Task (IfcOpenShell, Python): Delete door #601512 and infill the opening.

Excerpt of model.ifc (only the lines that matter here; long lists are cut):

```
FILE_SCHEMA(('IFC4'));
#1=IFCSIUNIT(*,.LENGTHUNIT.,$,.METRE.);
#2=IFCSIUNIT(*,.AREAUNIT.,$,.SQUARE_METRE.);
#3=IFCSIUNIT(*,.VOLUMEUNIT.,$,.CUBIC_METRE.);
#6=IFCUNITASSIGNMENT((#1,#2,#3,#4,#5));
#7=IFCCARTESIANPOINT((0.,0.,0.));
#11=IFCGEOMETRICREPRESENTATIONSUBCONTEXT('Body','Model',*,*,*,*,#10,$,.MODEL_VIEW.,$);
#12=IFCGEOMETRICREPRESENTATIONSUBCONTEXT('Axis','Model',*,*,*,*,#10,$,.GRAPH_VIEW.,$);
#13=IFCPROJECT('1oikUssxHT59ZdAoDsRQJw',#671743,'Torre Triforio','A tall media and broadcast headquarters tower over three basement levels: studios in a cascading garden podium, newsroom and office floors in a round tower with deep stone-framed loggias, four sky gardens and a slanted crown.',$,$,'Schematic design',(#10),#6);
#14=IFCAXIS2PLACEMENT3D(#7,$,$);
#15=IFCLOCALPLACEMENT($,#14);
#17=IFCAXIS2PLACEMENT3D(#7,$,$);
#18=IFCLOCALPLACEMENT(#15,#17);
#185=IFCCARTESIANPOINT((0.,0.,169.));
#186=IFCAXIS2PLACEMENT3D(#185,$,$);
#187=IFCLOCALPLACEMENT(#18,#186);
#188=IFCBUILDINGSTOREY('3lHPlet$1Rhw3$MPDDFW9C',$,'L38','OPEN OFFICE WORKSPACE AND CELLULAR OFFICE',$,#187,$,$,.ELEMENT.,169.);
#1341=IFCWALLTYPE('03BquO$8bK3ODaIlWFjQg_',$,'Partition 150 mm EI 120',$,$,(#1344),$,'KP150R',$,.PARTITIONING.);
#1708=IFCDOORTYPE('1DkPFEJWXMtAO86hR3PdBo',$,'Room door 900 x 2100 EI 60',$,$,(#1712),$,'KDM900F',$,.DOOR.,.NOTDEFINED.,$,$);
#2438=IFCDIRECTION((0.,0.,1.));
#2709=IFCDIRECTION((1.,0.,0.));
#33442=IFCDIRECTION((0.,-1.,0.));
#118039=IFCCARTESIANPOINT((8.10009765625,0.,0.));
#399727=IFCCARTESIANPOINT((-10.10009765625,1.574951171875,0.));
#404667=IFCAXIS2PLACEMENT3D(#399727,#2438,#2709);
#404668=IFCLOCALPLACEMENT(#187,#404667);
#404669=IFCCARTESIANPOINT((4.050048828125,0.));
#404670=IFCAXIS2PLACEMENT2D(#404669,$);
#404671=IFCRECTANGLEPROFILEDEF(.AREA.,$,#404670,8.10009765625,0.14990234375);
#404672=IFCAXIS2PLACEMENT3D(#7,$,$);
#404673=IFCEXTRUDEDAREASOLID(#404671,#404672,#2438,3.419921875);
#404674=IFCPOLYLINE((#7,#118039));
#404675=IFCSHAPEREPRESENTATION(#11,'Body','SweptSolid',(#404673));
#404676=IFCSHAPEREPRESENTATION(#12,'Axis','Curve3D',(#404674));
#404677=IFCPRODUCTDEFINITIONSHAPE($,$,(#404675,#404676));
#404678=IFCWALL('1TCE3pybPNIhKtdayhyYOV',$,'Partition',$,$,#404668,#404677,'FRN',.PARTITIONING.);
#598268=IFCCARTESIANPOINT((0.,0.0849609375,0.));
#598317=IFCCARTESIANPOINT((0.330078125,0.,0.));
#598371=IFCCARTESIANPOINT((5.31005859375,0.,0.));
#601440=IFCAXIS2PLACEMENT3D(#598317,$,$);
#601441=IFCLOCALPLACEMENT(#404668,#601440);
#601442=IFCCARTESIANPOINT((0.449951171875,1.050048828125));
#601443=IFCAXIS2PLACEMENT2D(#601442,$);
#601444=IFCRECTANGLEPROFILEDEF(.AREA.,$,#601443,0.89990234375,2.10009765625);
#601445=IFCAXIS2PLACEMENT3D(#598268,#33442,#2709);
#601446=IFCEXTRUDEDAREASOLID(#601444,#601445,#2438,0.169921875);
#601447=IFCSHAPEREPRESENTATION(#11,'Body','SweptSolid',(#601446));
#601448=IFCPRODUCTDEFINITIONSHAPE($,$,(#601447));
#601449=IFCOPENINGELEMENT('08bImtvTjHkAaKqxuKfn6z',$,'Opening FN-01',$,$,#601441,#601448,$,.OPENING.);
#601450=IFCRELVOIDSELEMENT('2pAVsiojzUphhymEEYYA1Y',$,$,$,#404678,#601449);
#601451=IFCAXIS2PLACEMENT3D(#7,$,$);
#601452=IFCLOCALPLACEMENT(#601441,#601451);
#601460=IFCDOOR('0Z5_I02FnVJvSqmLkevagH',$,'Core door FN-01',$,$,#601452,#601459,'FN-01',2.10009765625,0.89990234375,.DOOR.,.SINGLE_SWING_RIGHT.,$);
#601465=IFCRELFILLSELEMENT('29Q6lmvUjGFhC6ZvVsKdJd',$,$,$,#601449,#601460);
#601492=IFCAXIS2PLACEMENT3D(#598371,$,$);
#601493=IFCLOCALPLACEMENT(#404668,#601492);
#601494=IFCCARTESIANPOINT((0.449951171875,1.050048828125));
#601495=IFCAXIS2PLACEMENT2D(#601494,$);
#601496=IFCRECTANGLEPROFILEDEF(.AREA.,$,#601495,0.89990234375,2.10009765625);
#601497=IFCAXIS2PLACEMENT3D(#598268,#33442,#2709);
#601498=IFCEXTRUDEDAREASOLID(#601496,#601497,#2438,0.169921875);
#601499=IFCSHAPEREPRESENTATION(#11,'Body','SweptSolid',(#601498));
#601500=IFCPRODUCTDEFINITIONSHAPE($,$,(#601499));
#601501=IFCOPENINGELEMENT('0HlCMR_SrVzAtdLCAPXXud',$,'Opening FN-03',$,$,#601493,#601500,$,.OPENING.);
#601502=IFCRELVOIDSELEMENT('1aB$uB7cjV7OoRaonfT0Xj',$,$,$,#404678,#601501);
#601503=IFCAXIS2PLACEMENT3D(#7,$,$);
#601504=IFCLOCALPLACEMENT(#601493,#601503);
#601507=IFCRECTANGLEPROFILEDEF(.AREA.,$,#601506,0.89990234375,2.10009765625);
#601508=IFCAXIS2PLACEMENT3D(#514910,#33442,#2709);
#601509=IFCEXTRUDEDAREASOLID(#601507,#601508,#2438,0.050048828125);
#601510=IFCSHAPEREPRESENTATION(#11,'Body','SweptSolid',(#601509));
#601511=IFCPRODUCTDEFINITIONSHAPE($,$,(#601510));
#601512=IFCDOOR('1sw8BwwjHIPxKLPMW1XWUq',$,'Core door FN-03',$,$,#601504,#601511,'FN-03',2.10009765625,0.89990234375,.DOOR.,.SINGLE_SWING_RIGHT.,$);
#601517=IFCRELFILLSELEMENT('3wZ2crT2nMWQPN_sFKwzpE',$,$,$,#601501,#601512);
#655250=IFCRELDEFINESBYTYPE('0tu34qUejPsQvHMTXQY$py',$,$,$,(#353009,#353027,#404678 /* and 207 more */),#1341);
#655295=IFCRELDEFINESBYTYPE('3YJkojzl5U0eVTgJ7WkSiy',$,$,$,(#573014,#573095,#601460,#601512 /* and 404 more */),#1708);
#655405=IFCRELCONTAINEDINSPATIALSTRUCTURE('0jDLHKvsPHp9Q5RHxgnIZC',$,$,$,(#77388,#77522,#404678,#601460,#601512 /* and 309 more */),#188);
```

```python
import ifcopenshell
import ifcopenshell.api.feature
import ifcopenshell.api.root
import ifcopenshell.geom
import ifcopenshell.util.shape

model = ifcopenshell.open("model.ifc")
settings = ifcopenshell.geom.settings()


def volume(element):
    """Net volume in cubic metres, openings subtracted."""
    shape = ifcopenshell.geom.create_shape(settings, element)
    return ifcopenshell.util.shape.get_volume(shape.geometry)


door = model.by_guid("1sw8BwwjHIPxKLPMW1XWUq")
opening = door.FillsVoids[0].RelatingOpeningElement
wall = opening.VoidsElements[0].RelatingBuildingElement
before = volume(wall)

ifcopenshell.api.root.remove_product(model, product=door)
ifcopenshell.api.feature.remove_feature(model, feature=opening)

after = volume(wall)

print(f"wall volume {before:.3f} -> {after:.3f} m3")

model.write("model_edited.ifc")
```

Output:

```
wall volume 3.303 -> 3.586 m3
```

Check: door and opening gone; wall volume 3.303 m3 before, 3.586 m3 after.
